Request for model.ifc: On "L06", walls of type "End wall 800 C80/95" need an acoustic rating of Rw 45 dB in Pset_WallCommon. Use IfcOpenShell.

First a look at what the model holds.

```python
import ifcopenshell
import ifcopenshell.util.element

model = ifcopenshell.open("model.ifc")
print(model.schema)
storey = next(s for s in model.by_type("IfcBuildingStorey") if s.Name == "L06")
walls = [e for e in ifcopenshell.util.element.get_decomposition(storey) if e.is_a("IfcWall")]
seen = {}
for e in walls:
    element_type = ifcopenshell.util.element.get_type(e)
    key = (element_type.Name if element_type != e and element_type else None, ifcopenshell.util.element.get_pset(e, "Pset_WallCommon", "AcousticRating"))
    seen[key] = seen.get(key, 0) + 1
for (name, value), count in sorted(seen.items(), key=str):
    print(count, "x", name, "|", value)
```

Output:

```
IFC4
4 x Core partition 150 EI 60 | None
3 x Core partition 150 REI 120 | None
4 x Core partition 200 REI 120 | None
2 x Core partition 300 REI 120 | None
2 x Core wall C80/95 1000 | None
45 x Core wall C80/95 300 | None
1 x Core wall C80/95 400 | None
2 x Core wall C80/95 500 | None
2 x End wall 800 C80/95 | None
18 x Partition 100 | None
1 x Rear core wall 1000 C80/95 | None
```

```python
import ifcopenshell
import ifcopenshell.api.pset
import ifcopenshell.util.element

model = ifcopenshell.open("model.ifc")

storey = next(s for s in model.by_type("IfcBuildingStorey") if s.Name == "L06")
walls = [e for e in ifcopenshell.util.element.get_decomposition(storey) if e.is_a("IfcWall")]

count = 0
for e in walls:
    element_type = ifcopenshell.util.element.get_type(e)
    if element_type in (None, e) or element_type.Name != "End wall 800 C80/95":
        continue
    found = ifcopenshell.util.element.get_pset(e, "Pset_WallCommon", should_inherit=False)
    if found:
        pset = model.by_id(found["id"])
        if len(ifcopenshell.util.element.get_elements_by_pset(pset)) > 1:
            pset = ifcopenshell.api.pset.unshare_pset(model, products=[e], pset=pset)[0]
    else:
        pset = ifcopenshell.api.pset.add_pset(model, product=e, name="Pset_WallCommon")
    ifcopenshell.api.pset.edit_pset(model, pset=pset, properties={"AcousticRating": "Rw 45 dB"})
    count += 1

print(count, "walls updated")

model.write("model_rev.ifc")
```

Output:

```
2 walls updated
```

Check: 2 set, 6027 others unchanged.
